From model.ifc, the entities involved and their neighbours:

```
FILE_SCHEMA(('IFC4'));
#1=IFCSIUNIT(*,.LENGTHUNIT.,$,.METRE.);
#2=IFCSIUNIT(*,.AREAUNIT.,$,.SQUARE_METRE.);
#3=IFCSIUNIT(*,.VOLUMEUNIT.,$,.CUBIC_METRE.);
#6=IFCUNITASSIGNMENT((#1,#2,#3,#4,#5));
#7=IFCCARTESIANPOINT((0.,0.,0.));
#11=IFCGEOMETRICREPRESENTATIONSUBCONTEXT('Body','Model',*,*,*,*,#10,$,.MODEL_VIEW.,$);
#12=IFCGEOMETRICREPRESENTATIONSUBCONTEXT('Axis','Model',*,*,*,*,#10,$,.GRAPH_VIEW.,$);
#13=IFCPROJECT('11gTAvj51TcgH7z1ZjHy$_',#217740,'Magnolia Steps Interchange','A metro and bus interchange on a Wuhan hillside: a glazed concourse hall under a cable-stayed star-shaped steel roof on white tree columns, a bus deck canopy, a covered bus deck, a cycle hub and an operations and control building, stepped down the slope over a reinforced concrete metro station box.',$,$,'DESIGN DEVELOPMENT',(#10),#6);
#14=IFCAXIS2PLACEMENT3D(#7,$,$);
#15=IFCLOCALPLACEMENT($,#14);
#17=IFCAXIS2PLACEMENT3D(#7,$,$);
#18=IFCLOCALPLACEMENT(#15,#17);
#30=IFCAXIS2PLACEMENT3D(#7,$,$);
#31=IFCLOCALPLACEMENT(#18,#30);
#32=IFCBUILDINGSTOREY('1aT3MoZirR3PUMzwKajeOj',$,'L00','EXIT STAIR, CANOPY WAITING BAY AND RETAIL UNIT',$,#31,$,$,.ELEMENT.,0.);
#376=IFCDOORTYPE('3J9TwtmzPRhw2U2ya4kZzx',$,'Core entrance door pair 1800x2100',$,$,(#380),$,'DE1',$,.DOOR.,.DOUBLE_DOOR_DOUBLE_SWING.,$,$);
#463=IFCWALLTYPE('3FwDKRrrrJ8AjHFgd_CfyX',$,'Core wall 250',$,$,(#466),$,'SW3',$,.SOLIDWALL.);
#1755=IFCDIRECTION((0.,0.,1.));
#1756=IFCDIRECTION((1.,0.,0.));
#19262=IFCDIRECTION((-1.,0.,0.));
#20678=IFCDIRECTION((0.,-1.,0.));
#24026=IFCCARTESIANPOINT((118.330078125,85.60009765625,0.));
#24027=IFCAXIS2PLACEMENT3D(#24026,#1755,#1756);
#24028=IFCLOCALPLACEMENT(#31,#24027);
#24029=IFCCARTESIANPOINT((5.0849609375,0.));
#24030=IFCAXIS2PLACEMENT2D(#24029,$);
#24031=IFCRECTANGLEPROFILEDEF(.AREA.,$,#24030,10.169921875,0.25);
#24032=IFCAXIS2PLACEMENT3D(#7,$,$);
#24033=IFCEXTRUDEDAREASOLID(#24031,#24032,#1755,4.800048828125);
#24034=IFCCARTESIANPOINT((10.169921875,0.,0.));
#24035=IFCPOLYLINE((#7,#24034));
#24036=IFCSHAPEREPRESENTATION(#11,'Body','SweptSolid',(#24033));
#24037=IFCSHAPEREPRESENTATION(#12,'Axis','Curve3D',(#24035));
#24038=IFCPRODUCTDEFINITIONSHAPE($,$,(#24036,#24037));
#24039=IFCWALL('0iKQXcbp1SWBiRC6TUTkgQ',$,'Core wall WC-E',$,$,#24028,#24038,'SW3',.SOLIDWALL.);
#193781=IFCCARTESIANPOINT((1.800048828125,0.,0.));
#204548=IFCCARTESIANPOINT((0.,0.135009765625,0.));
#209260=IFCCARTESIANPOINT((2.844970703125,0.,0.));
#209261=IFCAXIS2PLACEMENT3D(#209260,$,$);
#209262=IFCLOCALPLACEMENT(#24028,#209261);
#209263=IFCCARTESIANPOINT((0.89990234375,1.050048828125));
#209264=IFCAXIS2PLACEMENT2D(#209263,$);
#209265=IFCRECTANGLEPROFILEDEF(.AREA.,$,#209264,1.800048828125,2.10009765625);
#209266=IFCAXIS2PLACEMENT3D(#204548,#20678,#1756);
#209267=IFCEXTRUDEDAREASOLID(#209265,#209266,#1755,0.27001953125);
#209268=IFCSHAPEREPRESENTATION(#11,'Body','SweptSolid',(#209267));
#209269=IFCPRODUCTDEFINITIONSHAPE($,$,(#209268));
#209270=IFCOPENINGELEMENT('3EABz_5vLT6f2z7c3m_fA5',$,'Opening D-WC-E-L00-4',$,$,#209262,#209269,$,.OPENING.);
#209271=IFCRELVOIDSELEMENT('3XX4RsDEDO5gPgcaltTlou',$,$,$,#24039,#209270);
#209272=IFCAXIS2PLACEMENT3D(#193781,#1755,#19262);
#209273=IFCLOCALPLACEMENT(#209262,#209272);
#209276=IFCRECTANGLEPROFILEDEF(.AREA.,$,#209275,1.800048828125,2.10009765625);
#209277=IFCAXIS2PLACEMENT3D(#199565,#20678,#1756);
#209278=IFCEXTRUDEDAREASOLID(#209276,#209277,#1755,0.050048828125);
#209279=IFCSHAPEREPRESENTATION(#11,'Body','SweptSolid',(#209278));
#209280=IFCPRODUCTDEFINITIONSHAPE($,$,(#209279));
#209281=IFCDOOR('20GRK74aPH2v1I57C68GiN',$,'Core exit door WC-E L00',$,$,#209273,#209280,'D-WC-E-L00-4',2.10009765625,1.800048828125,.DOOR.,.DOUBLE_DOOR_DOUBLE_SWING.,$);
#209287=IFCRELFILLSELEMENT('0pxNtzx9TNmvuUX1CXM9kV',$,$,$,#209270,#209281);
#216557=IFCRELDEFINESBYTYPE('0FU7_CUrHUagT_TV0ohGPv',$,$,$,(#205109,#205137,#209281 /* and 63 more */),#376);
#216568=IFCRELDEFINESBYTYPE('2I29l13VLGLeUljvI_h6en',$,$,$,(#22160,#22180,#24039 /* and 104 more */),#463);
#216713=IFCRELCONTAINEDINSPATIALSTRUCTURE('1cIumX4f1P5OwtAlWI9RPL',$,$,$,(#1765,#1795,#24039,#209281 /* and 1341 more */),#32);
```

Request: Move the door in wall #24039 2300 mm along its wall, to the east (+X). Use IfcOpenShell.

```python
import ifcopenshell
import ifcopenshell.api.geometry
import ifcopenshell.util.placement
import ifcopenshell.util.unit

model = ifcopenshell.open("model.ifc")
unit_scale = ifcopenshell.util.unit.calculate_unit_scale(model)

door = model.by_guid("20GRK74aPH2v1I57C68GiN")
opening = door.FillsVoids[0].RelatingOpeningElement
wall = opening.VoidsElements[0].RelatingBuildingElement

wall_matrix = ifcopenshell.util.placement.get_local_placement(wall.ObjectPlacement)
shift = wall_matrix[:3, 0] * 2.3 / unit_scale
before = ifcopenshell.util.placement.get_local_placement(door.ObjectPlacement)[:3, 3].copy()

# The door is placed relative to its opening, so it follows when the opening moves.
matrix = ifcopenshell.util.placement.get_local_placement(opening.ObjectPlacement)
matrix[:3, 3] += shift
ifcopenshell.api.geometry.edit_object_placement(
    model, product=opening, matrix=matrix, is_si=False, should_transform_children=True
)

after = ifcopenshell.util.placement.get_local_placement(door.ObjectPlacement)[:3, 3]
print("door moved by", (after - before).round(3) + 0.0)

model.write("model_edited.ifc")
```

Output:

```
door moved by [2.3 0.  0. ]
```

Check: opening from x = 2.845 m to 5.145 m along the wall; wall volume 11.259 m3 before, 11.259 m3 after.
